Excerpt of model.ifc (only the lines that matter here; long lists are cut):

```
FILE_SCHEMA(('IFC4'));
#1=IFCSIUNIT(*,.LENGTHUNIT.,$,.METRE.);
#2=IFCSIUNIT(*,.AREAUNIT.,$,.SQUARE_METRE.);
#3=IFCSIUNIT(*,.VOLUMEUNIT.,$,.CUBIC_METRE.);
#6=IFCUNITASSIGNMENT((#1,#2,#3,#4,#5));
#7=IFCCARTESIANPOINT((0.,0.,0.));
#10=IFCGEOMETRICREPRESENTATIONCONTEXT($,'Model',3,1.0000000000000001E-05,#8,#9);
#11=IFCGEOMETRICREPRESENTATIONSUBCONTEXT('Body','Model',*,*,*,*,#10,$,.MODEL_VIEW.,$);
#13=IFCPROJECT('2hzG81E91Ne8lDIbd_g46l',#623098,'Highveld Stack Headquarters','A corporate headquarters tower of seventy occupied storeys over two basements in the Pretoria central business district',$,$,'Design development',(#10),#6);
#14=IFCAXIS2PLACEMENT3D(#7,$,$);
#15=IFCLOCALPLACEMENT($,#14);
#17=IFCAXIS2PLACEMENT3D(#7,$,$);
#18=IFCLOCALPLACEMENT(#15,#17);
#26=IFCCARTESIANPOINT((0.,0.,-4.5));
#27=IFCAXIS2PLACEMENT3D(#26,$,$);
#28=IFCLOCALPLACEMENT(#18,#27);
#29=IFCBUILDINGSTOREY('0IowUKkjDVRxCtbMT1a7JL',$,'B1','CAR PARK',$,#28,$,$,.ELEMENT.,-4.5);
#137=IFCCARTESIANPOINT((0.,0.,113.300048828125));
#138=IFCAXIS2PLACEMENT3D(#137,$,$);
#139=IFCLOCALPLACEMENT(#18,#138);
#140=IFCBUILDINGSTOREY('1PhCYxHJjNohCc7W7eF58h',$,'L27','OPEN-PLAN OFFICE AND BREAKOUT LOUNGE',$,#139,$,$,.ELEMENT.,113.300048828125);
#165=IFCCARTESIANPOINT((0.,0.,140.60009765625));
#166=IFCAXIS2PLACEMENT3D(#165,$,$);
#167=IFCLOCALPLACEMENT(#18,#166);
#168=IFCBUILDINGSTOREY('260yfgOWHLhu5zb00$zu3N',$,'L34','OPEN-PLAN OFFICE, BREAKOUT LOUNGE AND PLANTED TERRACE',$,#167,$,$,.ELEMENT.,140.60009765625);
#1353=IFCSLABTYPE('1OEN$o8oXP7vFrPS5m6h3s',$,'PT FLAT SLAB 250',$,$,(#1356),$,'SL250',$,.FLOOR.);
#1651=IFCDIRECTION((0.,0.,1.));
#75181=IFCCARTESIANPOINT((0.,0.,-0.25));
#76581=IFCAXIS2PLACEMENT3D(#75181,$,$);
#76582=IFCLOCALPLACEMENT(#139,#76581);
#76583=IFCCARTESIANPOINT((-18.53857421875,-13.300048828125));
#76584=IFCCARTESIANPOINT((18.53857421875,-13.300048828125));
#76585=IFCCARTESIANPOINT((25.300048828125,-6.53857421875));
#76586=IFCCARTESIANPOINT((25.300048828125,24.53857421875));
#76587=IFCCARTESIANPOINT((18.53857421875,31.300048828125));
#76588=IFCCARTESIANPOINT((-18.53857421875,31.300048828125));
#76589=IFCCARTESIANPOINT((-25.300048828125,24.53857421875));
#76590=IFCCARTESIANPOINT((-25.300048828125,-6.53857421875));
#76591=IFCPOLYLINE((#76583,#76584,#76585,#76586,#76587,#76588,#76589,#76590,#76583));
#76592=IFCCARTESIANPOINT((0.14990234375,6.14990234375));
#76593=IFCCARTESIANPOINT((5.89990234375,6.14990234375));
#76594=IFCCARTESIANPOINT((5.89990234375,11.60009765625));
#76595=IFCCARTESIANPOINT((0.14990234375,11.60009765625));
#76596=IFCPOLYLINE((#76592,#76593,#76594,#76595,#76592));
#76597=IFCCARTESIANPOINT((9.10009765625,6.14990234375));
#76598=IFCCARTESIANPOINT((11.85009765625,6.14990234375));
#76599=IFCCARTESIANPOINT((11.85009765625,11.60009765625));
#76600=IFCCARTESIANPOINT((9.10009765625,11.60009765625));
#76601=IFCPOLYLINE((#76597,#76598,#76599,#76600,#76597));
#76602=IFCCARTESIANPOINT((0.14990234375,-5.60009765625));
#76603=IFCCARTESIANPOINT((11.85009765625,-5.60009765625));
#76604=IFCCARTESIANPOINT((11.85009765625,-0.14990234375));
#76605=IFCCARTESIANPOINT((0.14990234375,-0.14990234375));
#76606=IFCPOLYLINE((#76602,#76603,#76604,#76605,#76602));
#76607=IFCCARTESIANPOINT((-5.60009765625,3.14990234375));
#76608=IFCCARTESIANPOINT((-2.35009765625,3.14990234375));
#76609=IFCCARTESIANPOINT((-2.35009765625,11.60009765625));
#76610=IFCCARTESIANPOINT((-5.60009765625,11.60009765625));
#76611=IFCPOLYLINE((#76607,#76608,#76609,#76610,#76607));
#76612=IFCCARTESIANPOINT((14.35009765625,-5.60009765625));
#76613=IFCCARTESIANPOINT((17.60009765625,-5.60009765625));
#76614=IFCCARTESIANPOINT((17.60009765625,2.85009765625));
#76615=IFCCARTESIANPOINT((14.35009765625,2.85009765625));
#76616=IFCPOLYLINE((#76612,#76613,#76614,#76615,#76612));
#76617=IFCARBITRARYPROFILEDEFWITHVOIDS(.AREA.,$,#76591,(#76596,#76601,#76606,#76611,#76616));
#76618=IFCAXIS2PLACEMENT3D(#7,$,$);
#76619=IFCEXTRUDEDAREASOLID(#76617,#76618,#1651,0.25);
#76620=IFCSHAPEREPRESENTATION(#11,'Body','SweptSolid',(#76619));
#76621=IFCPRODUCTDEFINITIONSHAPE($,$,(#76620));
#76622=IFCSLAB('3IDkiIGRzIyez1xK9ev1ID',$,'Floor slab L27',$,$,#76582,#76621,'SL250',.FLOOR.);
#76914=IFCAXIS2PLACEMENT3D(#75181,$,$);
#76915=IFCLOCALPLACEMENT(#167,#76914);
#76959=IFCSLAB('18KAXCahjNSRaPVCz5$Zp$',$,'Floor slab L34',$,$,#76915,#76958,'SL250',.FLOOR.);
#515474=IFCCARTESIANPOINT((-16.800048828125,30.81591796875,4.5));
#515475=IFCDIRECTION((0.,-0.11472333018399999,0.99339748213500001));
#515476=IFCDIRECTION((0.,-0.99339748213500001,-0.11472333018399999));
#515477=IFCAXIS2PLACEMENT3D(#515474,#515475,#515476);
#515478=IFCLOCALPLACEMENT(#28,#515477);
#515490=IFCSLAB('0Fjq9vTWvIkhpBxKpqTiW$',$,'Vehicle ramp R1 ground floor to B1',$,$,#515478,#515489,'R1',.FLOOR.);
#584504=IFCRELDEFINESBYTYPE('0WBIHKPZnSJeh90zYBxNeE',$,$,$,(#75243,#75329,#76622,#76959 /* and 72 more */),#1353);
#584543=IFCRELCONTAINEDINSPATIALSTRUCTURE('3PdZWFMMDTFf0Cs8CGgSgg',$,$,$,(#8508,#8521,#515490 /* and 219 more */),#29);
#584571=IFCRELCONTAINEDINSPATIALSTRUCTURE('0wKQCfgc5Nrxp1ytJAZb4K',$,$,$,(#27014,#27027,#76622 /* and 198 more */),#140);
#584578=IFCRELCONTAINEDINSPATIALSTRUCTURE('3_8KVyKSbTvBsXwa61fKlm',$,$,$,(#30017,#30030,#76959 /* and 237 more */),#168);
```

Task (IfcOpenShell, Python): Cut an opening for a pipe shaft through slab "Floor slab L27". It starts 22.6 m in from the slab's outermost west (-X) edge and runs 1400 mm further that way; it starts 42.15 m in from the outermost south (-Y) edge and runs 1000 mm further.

```python
import numpy as np
import ifcopenshell
import ifcopenshell.api.feature
import ifcopenshell.api.geometry
import ifcopenshell.api.root
import ifcopenshell.geom
import ifcopenshell.util.placement
import ifcopenshell.util.representation
import ifcopenshell.util.shape
import ifcopenshell.util.unit

model = ifcopenshell.open("model.ifc")
unit_scale = ifcopenshell.util.unit.calculate_unit_scale(model)
settings = ifcopenshell.geom.settings()


def volume(element):
    """Net volume in cubic metres, openings subtracted."""
    shape = ifcopenshell.geom.create_shape(settings, element)
    return ifcopenshell.util.shape.get_volume(shape.geometry)


slab = model.by_id(76622)
before = volume(slab)

# Extent in the slab's own axes, in metres. The edges named are its -X and -Y sides.
slab_shape = ifcopenshell.geom.create_shape(settings, slab)
vertices = ifcopenshell.util.shape.get_vertices(slab_shape.geometry)
x_min, y_min, bottom = vertices.min(axis=0)
top = vertices[:, 2].max()

opening = ifcopenshell.api.root.create_entity(model, ifc_class="IfcOpeningElement", name="Pipe shaft opening", predefined_type="OPENING")
context = ifcopenshell.util.representation.get_context(model, "Model", "Body", "MODEL_VIEW")
width, depth = 1.4, 1
outline = [(0.0, 0.0), (width, 0.0), (width, depth), (0.0, depth), (0.0, 0.0)]
# Overshoot both faces by 50 mm so the cut is clean.
shape = ifcopenshell.api.geometry.add_slab_representation(
    model, context=context, depth=top - bottom + 0.1, polyline=outline
)
ifcopenshell.api.geometry.assign_representation(model, product=opening, representation=shape)

matrix = ifcopenshell.util.placement.get_local_placement(slab.ObjectPlacement)
matrix[:, 3] = matrix @ np.append(np.array([x_min + 22.6, y_min + 42.15, bottom - 0.05]) / unit_scale, 1.0)
ifcopenshell.api.geometry.edit_object_placement(model, product=opening, matrix=matrix, is_si=False)
ifcopenshell.api.feature.add_feature(model, feature=opening, element=slab)

after = volume(slab)

print(f"slab volume {before:.3f} -> {after:.3f} m3")

model.write("model_v2.ifc")
```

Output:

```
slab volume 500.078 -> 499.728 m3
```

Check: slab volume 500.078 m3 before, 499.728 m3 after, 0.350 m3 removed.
